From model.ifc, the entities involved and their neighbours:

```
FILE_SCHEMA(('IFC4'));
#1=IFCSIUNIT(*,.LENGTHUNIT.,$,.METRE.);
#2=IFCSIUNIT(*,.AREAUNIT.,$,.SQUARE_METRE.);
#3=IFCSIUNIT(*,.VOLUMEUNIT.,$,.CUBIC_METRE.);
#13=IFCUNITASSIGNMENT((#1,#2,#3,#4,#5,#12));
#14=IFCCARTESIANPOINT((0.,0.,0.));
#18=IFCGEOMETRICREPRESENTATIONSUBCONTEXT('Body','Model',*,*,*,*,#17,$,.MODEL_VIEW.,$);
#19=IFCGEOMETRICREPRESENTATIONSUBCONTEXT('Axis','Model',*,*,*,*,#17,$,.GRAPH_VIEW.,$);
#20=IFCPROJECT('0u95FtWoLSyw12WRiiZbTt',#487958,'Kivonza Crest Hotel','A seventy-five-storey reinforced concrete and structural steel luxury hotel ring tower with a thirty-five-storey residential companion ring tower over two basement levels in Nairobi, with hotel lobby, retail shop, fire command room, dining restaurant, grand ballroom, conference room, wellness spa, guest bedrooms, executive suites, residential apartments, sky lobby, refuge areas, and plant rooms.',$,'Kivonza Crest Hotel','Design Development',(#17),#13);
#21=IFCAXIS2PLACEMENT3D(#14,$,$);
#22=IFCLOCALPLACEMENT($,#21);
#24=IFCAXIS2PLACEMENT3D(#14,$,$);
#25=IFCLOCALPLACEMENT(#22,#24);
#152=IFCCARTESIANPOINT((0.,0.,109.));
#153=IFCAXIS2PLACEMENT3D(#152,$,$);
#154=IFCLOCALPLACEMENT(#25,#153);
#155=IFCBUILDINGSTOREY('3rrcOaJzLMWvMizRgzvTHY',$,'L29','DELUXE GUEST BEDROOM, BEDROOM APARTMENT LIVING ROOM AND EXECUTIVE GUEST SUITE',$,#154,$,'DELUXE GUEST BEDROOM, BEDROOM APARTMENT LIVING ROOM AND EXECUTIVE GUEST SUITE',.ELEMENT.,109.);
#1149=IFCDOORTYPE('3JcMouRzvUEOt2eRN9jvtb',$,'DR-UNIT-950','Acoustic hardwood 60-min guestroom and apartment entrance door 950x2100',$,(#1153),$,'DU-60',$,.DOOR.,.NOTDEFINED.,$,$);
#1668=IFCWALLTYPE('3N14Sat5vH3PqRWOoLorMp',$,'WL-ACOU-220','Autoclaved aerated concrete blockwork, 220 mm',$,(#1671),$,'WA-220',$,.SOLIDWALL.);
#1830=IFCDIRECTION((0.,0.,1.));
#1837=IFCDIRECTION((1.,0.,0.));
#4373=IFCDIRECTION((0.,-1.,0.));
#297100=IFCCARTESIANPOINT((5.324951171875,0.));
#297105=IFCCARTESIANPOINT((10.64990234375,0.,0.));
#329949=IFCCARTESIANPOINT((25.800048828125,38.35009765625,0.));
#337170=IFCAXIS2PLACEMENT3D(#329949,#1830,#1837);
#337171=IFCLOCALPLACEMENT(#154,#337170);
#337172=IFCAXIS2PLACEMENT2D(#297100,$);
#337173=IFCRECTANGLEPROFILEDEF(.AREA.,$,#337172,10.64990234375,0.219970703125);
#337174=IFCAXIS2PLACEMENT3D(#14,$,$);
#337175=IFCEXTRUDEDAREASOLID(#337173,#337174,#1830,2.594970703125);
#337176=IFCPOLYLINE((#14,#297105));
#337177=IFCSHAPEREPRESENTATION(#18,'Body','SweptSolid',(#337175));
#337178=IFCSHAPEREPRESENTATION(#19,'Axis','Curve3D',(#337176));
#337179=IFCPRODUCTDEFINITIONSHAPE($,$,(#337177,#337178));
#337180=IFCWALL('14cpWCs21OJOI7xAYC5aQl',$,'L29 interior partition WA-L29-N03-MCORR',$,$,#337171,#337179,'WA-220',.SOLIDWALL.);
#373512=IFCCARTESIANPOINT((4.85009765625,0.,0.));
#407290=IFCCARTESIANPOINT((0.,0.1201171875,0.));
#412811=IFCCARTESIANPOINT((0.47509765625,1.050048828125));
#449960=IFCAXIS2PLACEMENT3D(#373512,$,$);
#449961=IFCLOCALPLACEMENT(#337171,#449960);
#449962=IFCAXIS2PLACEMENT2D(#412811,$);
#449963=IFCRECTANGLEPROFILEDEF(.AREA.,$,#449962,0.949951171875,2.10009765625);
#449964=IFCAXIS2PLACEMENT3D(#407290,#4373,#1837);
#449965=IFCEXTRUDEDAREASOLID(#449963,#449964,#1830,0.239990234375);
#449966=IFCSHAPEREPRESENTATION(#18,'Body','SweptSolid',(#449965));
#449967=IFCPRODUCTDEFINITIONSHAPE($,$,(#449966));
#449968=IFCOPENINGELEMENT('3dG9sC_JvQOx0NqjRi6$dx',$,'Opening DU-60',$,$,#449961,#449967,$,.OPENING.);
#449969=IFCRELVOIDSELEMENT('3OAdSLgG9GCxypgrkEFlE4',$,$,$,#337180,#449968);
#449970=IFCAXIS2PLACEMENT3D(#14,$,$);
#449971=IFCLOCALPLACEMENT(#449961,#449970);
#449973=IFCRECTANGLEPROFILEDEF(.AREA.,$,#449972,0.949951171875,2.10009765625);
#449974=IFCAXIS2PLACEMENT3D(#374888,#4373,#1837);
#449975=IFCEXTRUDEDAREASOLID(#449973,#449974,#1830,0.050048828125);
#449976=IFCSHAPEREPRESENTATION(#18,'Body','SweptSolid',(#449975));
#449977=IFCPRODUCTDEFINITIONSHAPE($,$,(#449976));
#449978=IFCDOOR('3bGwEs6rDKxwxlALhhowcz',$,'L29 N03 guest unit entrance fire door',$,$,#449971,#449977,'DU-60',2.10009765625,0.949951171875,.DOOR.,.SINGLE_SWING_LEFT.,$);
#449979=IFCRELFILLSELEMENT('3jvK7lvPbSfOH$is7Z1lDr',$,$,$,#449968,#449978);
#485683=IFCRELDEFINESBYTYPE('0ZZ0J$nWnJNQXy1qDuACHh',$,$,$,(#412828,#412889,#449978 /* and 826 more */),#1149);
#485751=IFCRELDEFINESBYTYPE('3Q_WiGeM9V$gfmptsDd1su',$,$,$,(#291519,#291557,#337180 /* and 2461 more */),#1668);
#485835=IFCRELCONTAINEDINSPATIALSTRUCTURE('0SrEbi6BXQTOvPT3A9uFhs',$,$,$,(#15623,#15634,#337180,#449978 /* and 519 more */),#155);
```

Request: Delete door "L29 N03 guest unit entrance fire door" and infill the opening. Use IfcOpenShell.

```python
import ifcopenshell
import ifcopenshell.api.feature
import ifcopenshell.api.root
import ifcopenshell.geom
import ifcopenshell.util.shape

model = ifcopenshell.open("model.ifc")
settings = ifcopenshell.geom.settings()


def volume(element):
    """Net volume in cubic metres, openings subtracted."""
    shape = ifcopenshell.geom.create_shape(settings, element)
    return ifcopenshell.util.shape.get_volume(shape.geometry)


door = model.by_id(449978)
opening = door.FillsVoids[0].RelatingOpeningElement
wall = opening.VoidsElements[0].RelatingBuildingElement
before = volume(wall)

ifcopenshell.api.root.remove_product(model, product=door)
ifcopenshell.api.feature.remove_feature(model, feature=opening)

after = volume(wall)

print(f"wall volume {before:.3f} -> {after:.3f} m3")

model.write("model_rev.ifc")
```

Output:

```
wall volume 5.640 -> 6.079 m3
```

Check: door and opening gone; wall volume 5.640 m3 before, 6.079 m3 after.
